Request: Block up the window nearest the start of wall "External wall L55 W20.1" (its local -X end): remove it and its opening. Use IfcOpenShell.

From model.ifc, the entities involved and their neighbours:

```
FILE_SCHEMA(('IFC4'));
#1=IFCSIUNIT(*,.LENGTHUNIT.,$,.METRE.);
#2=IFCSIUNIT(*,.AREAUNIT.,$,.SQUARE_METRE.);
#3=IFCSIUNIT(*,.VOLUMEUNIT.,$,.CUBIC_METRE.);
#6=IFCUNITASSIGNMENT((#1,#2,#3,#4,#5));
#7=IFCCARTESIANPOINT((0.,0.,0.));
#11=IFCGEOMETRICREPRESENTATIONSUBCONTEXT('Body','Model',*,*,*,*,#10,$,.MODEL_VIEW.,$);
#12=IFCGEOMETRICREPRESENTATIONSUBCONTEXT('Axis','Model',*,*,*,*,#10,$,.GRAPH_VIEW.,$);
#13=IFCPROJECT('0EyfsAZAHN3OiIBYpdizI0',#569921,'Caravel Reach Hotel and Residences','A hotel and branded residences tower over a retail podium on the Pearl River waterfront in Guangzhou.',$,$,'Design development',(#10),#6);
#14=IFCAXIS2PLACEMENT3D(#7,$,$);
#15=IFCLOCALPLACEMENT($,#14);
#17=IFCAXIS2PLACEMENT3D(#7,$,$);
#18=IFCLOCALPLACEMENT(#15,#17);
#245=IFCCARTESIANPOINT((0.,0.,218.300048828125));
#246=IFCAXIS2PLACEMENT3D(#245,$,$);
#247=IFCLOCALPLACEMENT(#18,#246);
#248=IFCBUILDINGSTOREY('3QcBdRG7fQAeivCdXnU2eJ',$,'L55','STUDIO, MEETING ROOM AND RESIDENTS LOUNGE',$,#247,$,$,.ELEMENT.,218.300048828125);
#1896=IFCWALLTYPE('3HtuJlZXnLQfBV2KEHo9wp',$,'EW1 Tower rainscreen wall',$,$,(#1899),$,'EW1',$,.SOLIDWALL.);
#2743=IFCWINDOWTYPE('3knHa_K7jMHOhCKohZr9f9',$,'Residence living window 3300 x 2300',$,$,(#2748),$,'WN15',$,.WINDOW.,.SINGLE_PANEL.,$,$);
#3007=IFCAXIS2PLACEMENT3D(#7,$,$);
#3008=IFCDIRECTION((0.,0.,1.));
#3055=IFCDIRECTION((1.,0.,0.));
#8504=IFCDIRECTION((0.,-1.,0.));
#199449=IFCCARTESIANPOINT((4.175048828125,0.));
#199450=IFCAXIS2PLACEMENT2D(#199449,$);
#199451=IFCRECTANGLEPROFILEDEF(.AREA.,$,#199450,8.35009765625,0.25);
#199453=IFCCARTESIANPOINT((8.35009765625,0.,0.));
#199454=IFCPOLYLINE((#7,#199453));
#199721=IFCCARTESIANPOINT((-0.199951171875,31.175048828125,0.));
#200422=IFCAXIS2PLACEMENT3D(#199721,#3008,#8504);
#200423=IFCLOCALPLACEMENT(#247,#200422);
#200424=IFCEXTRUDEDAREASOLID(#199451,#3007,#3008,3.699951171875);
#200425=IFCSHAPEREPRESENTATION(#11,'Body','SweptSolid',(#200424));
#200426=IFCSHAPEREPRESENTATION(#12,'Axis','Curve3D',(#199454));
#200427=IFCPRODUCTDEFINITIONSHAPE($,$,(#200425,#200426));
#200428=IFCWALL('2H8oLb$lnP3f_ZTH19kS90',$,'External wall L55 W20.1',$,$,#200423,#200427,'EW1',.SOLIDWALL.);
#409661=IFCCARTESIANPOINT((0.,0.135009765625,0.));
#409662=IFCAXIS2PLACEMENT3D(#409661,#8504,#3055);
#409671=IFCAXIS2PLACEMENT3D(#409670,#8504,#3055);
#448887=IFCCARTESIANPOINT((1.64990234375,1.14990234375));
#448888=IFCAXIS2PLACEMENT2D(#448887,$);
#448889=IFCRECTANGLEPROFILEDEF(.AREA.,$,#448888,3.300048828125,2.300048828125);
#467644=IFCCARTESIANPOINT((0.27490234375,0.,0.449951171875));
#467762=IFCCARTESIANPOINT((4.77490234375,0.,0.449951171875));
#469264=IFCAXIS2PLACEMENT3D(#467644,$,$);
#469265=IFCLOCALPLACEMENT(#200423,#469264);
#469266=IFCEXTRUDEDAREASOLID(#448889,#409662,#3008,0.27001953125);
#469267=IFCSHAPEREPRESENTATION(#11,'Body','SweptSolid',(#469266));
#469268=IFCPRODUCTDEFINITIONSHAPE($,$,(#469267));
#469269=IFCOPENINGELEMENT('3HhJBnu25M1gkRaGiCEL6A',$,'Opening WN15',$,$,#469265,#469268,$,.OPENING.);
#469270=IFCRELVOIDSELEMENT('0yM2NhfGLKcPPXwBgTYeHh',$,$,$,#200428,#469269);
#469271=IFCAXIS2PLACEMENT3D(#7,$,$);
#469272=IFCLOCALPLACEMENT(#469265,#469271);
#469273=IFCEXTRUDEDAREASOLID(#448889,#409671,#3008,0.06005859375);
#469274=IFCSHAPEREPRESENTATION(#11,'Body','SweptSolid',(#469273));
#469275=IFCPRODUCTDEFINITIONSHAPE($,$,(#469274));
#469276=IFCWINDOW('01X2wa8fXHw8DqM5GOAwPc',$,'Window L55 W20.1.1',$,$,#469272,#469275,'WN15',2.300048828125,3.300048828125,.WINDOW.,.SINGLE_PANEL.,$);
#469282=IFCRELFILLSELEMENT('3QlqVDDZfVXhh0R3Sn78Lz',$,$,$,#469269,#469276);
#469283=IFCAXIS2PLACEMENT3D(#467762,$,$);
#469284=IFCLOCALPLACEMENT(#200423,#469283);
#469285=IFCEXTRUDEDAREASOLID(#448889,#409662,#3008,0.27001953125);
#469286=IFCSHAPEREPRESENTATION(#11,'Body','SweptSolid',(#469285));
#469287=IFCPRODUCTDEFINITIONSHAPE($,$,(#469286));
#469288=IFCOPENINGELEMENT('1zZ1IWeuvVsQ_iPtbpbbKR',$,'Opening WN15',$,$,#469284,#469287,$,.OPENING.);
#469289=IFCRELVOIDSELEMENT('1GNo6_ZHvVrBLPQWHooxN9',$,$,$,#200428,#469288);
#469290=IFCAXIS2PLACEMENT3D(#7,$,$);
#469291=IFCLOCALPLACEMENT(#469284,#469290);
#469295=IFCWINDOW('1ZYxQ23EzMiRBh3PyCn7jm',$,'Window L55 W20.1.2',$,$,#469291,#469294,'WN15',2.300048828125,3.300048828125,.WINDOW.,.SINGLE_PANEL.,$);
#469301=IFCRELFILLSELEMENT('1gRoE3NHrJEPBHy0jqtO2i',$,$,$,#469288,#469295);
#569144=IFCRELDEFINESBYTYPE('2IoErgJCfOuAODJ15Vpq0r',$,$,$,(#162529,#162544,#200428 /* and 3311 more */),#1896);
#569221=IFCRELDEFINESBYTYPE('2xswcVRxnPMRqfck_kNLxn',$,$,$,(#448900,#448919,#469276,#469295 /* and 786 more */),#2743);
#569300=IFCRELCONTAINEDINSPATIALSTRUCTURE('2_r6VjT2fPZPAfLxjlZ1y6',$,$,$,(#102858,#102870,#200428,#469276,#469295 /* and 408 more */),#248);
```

```python
import ifcopenshell
import ifcopenshell.api.feature
import ifcopenshell.api.root
import ifcopenshell.geom
import ifcopenshell.util.shape

model = ifcopenshell.open("model.ifc")
settings = ifcopenshell.geom.settings()


def volume(element):
    """Net volume in cubic metres, openings subtracted."""
    shape = ifcopenshell.geom.create_shape(settings, element)
    return ifcopenshell.util.shape.get_volume(shape.geometry)


window = model.by_guid("01X2wa8fXHw8DqM5GOAwPc")
opening = window.FillsVoids[0].RelatingOpeningElement
wall = opening.VoidsElements[0].RelatingBuildingElement
before = volume(wall)

ifcopenshell.api.root.remove_product(model, product=window)
ifcopenshell.api.feature.remove_feature(model, feature=opening)

after = volume(wall)

print(f"wall volume {before:.3f} -> {after:.3f} m3")

model.write("model-out.ifc")
```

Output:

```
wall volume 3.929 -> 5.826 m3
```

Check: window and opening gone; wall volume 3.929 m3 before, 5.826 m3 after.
